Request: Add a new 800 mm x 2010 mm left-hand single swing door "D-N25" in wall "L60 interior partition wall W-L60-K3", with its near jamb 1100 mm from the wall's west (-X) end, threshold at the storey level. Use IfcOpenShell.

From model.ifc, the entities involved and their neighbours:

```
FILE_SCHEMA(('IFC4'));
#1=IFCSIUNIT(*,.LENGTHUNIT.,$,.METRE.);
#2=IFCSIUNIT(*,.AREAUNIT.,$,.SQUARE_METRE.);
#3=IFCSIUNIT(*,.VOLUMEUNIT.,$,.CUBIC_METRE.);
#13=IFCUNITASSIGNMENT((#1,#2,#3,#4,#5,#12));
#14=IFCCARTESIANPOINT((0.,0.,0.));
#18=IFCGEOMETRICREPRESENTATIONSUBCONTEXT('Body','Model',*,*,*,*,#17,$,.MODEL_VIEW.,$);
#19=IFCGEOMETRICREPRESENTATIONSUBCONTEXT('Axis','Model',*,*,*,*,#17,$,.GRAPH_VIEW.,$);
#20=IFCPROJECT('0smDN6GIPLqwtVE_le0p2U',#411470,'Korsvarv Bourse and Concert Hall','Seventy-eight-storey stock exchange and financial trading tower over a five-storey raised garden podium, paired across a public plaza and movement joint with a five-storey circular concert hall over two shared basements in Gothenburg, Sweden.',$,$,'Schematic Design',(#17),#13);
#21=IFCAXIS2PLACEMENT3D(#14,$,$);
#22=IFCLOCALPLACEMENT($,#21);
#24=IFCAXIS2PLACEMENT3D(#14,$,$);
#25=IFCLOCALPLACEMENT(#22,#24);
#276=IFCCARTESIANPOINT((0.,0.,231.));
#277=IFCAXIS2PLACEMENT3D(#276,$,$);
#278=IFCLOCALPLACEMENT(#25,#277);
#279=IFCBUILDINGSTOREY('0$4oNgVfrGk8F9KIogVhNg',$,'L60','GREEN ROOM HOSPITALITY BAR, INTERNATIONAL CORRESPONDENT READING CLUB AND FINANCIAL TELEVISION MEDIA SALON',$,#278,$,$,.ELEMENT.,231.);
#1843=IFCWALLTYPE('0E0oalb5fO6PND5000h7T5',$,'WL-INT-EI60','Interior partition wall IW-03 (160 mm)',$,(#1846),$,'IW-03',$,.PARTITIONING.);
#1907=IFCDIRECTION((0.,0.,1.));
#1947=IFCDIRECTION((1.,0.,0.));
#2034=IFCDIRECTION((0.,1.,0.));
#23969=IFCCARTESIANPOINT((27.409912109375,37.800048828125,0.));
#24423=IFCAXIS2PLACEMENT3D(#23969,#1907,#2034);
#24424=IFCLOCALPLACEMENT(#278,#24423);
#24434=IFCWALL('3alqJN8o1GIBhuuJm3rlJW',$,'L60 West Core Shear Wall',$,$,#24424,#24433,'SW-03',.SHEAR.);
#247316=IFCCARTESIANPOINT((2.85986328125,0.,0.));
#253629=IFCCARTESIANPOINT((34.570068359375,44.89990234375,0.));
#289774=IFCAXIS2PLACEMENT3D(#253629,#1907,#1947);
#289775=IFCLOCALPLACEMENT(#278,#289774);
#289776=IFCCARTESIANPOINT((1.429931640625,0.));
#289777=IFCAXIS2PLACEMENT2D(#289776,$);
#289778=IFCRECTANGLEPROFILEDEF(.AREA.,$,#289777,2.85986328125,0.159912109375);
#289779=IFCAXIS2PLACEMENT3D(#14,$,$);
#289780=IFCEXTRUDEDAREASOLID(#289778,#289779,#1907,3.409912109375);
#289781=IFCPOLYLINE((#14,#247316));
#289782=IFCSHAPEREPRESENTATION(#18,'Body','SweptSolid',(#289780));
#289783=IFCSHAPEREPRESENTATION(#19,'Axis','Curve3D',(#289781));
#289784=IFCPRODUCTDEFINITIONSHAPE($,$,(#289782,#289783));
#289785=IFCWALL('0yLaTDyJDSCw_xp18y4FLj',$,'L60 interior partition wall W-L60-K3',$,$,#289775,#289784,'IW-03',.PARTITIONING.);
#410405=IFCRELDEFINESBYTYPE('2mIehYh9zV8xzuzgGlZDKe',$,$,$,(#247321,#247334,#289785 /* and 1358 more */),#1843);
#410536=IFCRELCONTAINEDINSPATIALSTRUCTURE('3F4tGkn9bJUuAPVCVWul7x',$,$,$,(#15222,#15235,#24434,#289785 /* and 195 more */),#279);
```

```python
import numpy as np
import ifcopenshell
import ifcopenshell.api.feature
import ifcopenshell.api.geometry
import ifcopenshell.api.root
import ifcopenshell.api.spatial
import ifcopenshell.geom
import ifcopenshell.util.element
import ifcopenshell.util.placement
import ifcopenshell.util.representation
import ifcopenshell.util.shape
import ifcopenshell.util.unit

model = ifcopenshell.open("model.ifc")
unit_scale = ifcopenshell.util.unit.calculate_unit_scale(model)
settings = ifcopenshell.geom.settings()


def volume(element):
    """Net volume in cubic metres, openings subtracted."""
    shape = ifcopenshell.geom.create_shape(settings, element)
    return ifcopenshell.util.shape.get_volume(shape.geometry)


wall = model.by_guid("0yLaTDyJDSCw_xp18y4FLj")
storey = ifcopenshell.util.element.get_container(wall, ifc_class="IfcBuildingStorey")
context = ifcopenshell.util.representation.get_context(model, "Model", "Body", "MODEL_VIEW")
before = volume(wall)

width, height, from_end, sill = 0.8, 2.01, 1.1, 0.0  # metres

# The wall runs along its own X axis, and the end named is its -X end.
wall_shape = ifcopenshell.geom.create_shape(settings, wall)
x, y, z = ifcopenshell.util.shape.get_vertices(wall_shape.geometry).T
start = x.min() + from_end
face, thickness = float(y.min()), float(y.max() - y.min())
wall_matrix = ifcopenshell.util.placement.get_local_placement(wall.ObjectPlacement)
level = ifcopenshell.util.placement.get_local_placement(storey.ObjectPlacement)[2, 3]


def in_wall(x, y):
    """Placement at x, y metres in the wall's axes, at sill height."""
    matrix = wall_matrix.copy()
    matrix[:, 3] = wall_matrix @ np.array([x / unit_scale, y / unit_scale, 0.0, 1.0])
    matrix[2, 3] = level + sill / unit_scale
    return matrix


# Opening: a box that overshoots both wall faces by 50 mm.
opening = ifcopenshell.api.root.create_entity(model, ifc_class="IfcOpeningElement", predefined_type="OPENING")
box = ifcopenshell.api.geometry.add_wall_representation(
    model, context=context, length=width, height=height, thickness=thickness + 0.1
)
ifcopenshell.api.geometry.assign_representation(model, product=opening, representation=box)
ifcopenshell.api.geometry.edit_object_placement(model, product=opening, matrix=in_wall(start, face - 0.05), is_si=False)
ifcopenshell.api.feature.add_feature(model, feature=opening, element=wall)

door = ifcopenshell.api.root.create_entity(model, ifc_class="IfcDoor", name="D-N25", predefined_type="DOOR")
door.OverallWidth, door.OverallHeight = width / unit_scale, height / unit_scale
door.OperationType = "SINGLE_SWING_LEFT"
body = ifcopenshell.api.geometry.add_door_representation(
    model,
    context=context,
    overall_width=door.OverallWidth,
    overall_height=door.OverallHeight,
    operation_type="SINGLE_SWING_LEFT",
    lining_properties={"LiningDepth": thickness / unit_scale, "ThresholdDepth": thickness / unit_scale},
)
ifcopenshell.api.geometry.assign_representation(model, product=door, representation=body)
ifcopenshell.api.spatial.assign_container(model, products=[door], relating_structure=storey)
ifcopenshell.api.feature.add_filling(model, opening=opening, element=door)

# The lining spans the wall, so the door starts at the wall face.
ifcopenshell.api.geometry.edit_object_placement(model, product=door, matrix=in_wall(start, face), is_si=False)

after = volume(wall)

print(f"wall volume {before:.3f} -> {after:.3f} m3")

model.write("model_edited.ifc")
```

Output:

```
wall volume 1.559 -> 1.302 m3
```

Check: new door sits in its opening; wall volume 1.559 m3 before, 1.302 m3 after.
